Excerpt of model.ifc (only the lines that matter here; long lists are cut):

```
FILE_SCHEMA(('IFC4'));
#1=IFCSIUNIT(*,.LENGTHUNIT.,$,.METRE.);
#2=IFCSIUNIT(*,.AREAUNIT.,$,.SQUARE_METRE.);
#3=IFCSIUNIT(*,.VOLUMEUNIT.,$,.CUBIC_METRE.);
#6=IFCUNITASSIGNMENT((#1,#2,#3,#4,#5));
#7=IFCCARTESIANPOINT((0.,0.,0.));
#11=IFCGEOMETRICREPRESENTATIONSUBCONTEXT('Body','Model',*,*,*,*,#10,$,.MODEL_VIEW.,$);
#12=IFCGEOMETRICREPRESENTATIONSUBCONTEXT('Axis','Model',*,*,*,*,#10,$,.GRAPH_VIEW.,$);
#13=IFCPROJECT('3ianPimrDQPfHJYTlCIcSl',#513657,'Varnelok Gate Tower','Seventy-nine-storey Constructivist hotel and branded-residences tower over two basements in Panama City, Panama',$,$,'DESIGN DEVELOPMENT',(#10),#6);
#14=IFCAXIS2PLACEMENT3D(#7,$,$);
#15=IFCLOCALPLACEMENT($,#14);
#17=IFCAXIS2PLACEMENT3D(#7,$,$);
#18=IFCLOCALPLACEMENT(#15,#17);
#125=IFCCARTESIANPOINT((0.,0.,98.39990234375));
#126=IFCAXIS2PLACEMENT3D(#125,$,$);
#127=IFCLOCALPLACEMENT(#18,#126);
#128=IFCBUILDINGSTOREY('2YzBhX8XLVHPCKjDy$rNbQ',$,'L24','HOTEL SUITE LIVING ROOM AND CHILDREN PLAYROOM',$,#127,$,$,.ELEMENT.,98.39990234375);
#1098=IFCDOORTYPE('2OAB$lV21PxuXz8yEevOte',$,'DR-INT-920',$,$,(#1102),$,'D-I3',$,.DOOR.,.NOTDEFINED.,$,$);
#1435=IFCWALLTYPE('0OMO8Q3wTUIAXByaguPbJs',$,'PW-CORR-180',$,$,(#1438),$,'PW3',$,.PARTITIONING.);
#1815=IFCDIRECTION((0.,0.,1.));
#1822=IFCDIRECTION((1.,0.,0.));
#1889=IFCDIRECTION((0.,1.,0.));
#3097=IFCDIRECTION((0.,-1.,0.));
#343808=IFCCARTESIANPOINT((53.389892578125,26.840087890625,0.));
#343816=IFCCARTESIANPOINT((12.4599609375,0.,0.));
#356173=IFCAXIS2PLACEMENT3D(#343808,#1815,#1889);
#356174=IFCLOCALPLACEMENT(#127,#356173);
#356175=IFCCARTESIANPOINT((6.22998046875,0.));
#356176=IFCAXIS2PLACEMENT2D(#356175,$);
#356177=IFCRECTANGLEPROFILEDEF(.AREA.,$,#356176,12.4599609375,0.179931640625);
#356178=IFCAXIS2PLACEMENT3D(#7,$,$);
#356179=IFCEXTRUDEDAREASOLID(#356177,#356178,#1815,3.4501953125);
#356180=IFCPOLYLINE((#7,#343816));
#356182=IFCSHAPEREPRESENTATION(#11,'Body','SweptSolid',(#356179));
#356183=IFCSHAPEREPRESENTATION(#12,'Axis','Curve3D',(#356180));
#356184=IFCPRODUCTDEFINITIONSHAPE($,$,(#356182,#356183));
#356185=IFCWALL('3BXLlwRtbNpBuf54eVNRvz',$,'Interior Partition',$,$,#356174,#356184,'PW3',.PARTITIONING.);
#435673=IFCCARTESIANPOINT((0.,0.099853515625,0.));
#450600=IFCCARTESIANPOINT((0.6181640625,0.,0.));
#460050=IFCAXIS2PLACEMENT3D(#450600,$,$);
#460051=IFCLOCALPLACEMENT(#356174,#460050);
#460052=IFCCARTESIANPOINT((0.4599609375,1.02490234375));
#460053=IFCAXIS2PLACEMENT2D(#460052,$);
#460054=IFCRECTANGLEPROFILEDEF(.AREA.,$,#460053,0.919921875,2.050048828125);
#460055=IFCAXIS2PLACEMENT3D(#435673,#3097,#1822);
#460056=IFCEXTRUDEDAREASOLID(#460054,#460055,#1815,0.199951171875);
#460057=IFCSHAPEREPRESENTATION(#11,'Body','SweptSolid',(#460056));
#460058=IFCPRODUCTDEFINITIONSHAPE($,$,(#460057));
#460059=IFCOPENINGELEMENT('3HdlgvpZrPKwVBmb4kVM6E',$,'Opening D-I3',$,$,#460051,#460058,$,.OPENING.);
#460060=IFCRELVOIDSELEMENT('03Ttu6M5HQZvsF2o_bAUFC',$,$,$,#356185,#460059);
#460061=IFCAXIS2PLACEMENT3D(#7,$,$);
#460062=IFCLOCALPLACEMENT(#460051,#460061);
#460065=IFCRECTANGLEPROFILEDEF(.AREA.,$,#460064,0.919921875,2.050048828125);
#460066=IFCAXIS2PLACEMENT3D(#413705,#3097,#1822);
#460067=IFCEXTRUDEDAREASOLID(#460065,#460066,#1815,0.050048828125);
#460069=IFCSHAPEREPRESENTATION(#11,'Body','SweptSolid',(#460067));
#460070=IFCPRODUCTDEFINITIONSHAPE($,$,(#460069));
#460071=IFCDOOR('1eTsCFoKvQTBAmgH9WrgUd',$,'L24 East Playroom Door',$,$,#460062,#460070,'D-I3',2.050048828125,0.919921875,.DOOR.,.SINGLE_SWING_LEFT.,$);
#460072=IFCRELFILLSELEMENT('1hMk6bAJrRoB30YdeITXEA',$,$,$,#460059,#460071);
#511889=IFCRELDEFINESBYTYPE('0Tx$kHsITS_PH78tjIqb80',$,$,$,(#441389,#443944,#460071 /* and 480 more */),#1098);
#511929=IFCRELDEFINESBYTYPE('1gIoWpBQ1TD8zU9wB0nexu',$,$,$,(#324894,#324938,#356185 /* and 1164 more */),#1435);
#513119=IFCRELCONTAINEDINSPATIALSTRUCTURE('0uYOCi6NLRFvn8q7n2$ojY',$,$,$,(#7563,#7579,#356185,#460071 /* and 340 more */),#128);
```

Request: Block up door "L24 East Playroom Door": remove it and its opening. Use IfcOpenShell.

```python
import ifcopenshell
import ifcopenshell.api.feature
import ifcopenshell.api.root
import ifcopenshell.geom
import ifcopenshell.util.shape

model = ifcopenshell.open("model.ifc")
settings = ifcopenshell.geom.settings()


def volume(element):
    """Net volume in cubic metres, openings subtracted."""
    shape = ifcopenshell.geom.create_shape(settings, element)
    return ifcopenshell.util.shape.get_volume(shape.geometry)


door = model.by_guid("1eTsCFoKvQTBAmgH9WrgUd")
opening = door.FillsVoids[0].RelatingOpeningElement
wall = opening.VoidsElements[0].RelatingBuildingElement
before = volume(wall)

ifcopenshell.api.root.remove_product(model, product=door)
ifcopenshell.api.feature.remove_feature(model, feature=opening)

after = volume(wall)

print(f"wall volume {before:.3f} -> {after:.3f} m3")

model.write("model_updated.ifc")
```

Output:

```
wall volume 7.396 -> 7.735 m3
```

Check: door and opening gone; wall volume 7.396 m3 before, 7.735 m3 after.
